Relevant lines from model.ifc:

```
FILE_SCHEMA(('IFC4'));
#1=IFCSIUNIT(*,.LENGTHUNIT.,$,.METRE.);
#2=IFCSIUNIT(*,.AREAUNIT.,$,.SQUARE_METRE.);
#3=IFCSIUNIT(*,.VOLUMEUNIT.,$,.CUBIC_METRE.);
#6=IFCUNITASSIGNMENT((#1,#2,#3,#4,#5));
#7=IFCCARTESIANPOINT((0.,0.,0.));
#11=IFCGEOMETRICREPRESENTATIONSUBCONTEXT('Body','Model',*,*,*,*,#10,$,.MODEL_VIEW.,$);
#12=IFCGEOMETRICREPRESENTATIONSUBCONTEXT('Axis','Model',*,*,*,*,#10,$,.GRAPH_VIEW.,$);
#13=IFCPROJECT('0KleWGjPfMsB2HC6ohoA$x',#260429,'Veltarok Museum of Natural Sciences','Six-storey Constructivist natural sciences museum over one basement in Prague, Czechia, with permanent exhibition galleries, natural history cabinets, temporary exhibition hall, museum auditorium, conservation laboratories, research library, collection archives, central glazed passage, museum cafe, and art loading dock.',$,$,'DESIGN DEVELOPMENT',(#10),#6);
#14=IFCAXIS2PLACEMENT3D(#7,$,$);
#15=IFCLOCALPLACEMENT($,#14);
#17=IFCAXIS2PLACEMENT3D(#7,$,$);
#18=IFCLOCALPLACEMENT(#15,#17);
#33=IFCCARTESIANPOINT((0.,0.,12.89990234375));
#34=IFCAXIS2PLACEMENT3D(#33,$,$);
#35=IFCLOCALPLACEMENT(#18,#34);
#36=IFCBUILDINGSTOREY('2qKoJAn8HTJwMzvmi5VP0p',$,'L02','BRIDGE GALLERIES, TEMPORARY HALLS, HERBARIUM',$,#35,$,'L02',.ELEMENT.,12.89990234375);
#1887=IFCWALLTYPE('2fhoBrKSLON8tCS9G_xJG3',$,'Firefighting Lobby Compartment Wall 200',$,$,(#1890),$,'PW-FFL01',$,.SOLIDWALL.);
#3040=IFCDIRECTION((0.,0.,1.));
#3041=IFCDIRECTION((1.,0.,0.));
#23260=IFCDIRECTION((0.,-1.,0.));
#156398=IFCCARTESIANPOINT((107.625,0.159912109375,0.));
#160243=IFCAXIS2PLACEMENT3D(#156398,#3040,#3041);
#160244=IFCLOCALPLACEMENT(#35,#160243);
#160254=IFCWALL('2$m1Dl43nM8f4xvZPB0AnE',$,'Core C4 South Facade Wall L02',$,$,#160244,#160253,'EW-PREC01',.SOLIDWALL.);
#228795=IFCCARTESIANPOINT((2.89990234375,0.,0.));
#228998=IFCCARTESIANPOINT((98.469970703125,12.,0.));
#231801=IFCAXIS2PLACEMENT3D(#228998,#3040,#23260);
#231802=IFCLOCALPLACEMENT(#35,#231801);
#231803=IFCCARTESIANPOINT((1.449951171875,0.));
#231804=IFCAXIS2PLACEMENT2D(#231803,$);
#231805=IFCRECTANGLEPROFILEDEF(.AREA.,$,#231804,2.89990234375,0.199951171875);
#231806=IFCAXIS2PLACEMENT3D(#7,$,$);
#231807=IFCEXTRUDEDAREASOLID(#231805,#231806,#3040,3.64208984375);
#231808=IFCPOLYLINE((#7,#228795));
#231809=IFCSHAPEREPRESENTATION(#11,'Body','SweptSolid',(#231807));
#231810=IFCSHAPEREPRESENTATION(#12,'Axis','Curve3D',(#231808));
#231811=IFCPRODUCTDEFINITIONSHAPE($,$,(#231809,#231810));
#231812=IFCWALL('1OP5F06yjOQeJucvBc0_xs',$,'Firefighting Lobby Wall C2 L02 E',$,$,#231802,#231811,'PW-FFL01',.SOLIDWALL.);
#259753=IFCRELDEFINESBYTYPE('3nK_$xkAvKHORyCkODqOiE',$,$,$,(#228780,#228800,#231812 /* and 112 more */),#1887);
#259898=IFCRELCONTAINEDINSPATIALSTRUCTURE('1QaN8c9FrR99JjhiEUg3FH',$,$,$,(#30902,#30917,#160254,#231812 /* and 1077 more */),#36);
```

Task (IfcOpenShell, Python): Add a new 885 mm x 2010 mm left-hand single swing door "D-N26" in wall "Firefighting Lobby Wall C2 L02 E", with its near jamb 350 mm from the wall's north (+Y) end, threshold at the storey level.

```python
import numpy as np
import ifcopenshell
import ifcopenshell.api.feature
import ifcopenshell.api.geometry
import ifcopenshell.api.root
import ifcopenshell.api.spatial
import ifcopenshell.geom
import ifcopenshell.util.element
import ifcopenshell.util.placement
import ifcopenshell.util.representation
import ifcopenshell.util.shape
import ifcopenshell.util.unit

model = ifcopenshell.open("model.ifc")
unit_scale = ifcopenshell.util.unit.calculate_unit_scale(model)
settings = ifcopenshell.geom.settings()


def volume(element):
    """Net volume in cubic metres, openings subtracted."""
    shape = ifcopenshell.geom.create_shape(settings, element)
    return ifcopenshell.util.shape.get_volume(shape.geometry)


wall = model.by_guid("1OP5F06yjOQeJucvBc0_xs")
storey = ifcopenshell.util.element.get_container(wall, ifc_class="IfcBuildingStorey")
context = ifcopenshell.util.representation.get_context(model, "Model", "Body", "MODEL_VIEW")
before = volume(wall)

width, height, from_end, sill = 0.885, 2.01, 0.35, 0.0  # metres

# The wall runs along its own X axis, and the end named is its -X end.
wall_shape = ifcopenshell.geom.create_shape(settings, wall)
x, y, z = ifcopenshell.util.shape.get_vertices(wall_shape.geometry).T
start = x.min() + from_end
face, thickness = float(y.min()), float(y.max() - y.min())
wall_matrix = ifcopenshell.util.placement.get_local_placement(wall.ObjectPlacement)
level = ifcopenshell.util.placement.get_local_placement(storey.ObjectPlacement)[2, 3]


def in_wall(x, y):
    """Placement at x, y metres in the wall's axes, at sill height."""
    matrix = wall_matrix.copy()
    matrix[:, 3] = wall_matrix @ np.array([x / unit_scale, y / unit_scale, 0.0, 1.0])
    matrix[2, 3] = level + sill / unit_scale
    return matrix


# Opening: a box that overshoots both wall faces by 50 mm.
opening = ifcopenshell.api.root.create_entity(model, ifc_class="IfcOpeningElement", predefined_type="OPENING")
box = ifcopenshell.api.geometry.add_wall_representation(
    model, context=context, length=width, height=height, thickness=thickness + 0.1
)
ifcopenshell.api.geometry.assign_representation(model, product=opening, representation=box)
ifcopenshell.api.geometry.edit_object_placement(model, product=opening, matrix=in_wall(start, face - 0.05), is_si=False)
ifcopenshell.api.feature.add_feature(model, feature=opening, element=wall)

door = ifcopenshell.api.root.create_entity(model, ifc_class="IfcDoor", name="D-N26", predefined_type="DOOR")
door.OverallWidth, door.OverallHeight = width / unit_scale, height / unit_scale
door.OperationType = "SINGLE_SWING_LEFT"
body = ifcopenshell.api.geometry.add_door_representation(
    model,
    context=context,
    overall_width=door.OverallWidth,
    overall_height=door.OverallHeight,
    operation_type="SINGLE_SWING_LEFT",
    lining_properties={"LiningDepth": thickness / unit_scale, "ThresholdDepth": thickness / unit_scale},
)
ifcopenshell.api.geometry.assign_representation(model, product=door, representation=body)
ifcopenshell.api.spatial.assign_container(model, products=[door], relating_structure=storey)
ifcopenshell.api.feature.add_filling(model, opening=opening, element=door)

# The lining spans the wall, so the door starts at the wall face.
ifcopenshell.api.geometry.edit_object_placement(model, product=door, matrix=in_wall(start, face), is_si=False)

after = volume(wall)

print(f"wall volume {before:.3f} -> {after:.3f} m3")

model.write("model_rev.ifc")
```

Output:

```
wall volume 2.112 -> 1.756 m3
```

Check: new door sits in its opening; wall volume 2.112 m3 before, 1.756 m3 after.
